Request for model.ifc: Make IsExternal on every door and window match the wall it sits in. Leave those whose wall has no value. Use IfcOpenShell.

First a look at what the model holds.

```python
import ifcopenshell
import ifcopenshell.util.element

model = ifcopenshell.open("model.ifc")
print(model.schema)
seen = {}
for e in model.by_type("IfcDoor") + model.by_type("IfcWindow"):
    if not e.FillsVoids:
        continue
    host = e.FillsVoids[0].RelatingOpeningElement.VoidsElements[0].RelatingBuildingElement
    own = ifcopenshell.util.element.get_pset(e, f"Pset_{e.is_a()[3:].removesuffix('StandardCase')}Common", "IsExternal")
    wall = ifcopenshell.util.element.get_pset(host, "Pset_WallCommon", "IsExternal")
    seen[e.is_a(), own, wall] = seen.get((e.is_a(), own, wall), 0) + 1
for (cls, own, wall), count in sorted(seen.items(), key=str):
    print(count, cls, "IsExternal:", own, "| host wall:", wall)
```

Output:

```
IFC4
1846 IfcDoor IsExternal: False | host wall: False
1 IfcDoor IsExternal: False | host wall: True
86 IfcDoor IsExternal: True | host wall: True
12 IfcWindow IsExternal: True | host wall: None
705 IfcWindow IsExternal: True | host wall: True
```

```python
import ifcopenshell
import ifcopenshell.api.pset
import ifcopenshell.util.element

model = ifcopenshell.open("model.ifc")

count = 0
for ifc_class, pset_name in (("IfcDoor", "Pset_DoorCommon"), ("IfcWindow", "Pset_WindowCommon")):
    for e in model.by_type(ifc_class):
        if not e.FillsVoids:
            continue
        host = e.FillsVoids[0].RelatingOpeningElement.VoidsElements[0].RelatingBuildingElement
        external = ifcopenshell.util.element.get_pset(host, "Pset_WallCommon", "IsExternal")
        if external is None or ifcopenshell.util.element.get_pset(e, pset_name, "IsExternal") == external:
            continue
        pset = ifcopenshell.api.pset.add_pset(model, product=e, name=pset_name)
        ifcopenshell.api.pset.edit_pset(model, pset=pset, properties={"IsExternal": external})
        count += 1

print(count, "updated")

model.write("model_v2.ifc")
```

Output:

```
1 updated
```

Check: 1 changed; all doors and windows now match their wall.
